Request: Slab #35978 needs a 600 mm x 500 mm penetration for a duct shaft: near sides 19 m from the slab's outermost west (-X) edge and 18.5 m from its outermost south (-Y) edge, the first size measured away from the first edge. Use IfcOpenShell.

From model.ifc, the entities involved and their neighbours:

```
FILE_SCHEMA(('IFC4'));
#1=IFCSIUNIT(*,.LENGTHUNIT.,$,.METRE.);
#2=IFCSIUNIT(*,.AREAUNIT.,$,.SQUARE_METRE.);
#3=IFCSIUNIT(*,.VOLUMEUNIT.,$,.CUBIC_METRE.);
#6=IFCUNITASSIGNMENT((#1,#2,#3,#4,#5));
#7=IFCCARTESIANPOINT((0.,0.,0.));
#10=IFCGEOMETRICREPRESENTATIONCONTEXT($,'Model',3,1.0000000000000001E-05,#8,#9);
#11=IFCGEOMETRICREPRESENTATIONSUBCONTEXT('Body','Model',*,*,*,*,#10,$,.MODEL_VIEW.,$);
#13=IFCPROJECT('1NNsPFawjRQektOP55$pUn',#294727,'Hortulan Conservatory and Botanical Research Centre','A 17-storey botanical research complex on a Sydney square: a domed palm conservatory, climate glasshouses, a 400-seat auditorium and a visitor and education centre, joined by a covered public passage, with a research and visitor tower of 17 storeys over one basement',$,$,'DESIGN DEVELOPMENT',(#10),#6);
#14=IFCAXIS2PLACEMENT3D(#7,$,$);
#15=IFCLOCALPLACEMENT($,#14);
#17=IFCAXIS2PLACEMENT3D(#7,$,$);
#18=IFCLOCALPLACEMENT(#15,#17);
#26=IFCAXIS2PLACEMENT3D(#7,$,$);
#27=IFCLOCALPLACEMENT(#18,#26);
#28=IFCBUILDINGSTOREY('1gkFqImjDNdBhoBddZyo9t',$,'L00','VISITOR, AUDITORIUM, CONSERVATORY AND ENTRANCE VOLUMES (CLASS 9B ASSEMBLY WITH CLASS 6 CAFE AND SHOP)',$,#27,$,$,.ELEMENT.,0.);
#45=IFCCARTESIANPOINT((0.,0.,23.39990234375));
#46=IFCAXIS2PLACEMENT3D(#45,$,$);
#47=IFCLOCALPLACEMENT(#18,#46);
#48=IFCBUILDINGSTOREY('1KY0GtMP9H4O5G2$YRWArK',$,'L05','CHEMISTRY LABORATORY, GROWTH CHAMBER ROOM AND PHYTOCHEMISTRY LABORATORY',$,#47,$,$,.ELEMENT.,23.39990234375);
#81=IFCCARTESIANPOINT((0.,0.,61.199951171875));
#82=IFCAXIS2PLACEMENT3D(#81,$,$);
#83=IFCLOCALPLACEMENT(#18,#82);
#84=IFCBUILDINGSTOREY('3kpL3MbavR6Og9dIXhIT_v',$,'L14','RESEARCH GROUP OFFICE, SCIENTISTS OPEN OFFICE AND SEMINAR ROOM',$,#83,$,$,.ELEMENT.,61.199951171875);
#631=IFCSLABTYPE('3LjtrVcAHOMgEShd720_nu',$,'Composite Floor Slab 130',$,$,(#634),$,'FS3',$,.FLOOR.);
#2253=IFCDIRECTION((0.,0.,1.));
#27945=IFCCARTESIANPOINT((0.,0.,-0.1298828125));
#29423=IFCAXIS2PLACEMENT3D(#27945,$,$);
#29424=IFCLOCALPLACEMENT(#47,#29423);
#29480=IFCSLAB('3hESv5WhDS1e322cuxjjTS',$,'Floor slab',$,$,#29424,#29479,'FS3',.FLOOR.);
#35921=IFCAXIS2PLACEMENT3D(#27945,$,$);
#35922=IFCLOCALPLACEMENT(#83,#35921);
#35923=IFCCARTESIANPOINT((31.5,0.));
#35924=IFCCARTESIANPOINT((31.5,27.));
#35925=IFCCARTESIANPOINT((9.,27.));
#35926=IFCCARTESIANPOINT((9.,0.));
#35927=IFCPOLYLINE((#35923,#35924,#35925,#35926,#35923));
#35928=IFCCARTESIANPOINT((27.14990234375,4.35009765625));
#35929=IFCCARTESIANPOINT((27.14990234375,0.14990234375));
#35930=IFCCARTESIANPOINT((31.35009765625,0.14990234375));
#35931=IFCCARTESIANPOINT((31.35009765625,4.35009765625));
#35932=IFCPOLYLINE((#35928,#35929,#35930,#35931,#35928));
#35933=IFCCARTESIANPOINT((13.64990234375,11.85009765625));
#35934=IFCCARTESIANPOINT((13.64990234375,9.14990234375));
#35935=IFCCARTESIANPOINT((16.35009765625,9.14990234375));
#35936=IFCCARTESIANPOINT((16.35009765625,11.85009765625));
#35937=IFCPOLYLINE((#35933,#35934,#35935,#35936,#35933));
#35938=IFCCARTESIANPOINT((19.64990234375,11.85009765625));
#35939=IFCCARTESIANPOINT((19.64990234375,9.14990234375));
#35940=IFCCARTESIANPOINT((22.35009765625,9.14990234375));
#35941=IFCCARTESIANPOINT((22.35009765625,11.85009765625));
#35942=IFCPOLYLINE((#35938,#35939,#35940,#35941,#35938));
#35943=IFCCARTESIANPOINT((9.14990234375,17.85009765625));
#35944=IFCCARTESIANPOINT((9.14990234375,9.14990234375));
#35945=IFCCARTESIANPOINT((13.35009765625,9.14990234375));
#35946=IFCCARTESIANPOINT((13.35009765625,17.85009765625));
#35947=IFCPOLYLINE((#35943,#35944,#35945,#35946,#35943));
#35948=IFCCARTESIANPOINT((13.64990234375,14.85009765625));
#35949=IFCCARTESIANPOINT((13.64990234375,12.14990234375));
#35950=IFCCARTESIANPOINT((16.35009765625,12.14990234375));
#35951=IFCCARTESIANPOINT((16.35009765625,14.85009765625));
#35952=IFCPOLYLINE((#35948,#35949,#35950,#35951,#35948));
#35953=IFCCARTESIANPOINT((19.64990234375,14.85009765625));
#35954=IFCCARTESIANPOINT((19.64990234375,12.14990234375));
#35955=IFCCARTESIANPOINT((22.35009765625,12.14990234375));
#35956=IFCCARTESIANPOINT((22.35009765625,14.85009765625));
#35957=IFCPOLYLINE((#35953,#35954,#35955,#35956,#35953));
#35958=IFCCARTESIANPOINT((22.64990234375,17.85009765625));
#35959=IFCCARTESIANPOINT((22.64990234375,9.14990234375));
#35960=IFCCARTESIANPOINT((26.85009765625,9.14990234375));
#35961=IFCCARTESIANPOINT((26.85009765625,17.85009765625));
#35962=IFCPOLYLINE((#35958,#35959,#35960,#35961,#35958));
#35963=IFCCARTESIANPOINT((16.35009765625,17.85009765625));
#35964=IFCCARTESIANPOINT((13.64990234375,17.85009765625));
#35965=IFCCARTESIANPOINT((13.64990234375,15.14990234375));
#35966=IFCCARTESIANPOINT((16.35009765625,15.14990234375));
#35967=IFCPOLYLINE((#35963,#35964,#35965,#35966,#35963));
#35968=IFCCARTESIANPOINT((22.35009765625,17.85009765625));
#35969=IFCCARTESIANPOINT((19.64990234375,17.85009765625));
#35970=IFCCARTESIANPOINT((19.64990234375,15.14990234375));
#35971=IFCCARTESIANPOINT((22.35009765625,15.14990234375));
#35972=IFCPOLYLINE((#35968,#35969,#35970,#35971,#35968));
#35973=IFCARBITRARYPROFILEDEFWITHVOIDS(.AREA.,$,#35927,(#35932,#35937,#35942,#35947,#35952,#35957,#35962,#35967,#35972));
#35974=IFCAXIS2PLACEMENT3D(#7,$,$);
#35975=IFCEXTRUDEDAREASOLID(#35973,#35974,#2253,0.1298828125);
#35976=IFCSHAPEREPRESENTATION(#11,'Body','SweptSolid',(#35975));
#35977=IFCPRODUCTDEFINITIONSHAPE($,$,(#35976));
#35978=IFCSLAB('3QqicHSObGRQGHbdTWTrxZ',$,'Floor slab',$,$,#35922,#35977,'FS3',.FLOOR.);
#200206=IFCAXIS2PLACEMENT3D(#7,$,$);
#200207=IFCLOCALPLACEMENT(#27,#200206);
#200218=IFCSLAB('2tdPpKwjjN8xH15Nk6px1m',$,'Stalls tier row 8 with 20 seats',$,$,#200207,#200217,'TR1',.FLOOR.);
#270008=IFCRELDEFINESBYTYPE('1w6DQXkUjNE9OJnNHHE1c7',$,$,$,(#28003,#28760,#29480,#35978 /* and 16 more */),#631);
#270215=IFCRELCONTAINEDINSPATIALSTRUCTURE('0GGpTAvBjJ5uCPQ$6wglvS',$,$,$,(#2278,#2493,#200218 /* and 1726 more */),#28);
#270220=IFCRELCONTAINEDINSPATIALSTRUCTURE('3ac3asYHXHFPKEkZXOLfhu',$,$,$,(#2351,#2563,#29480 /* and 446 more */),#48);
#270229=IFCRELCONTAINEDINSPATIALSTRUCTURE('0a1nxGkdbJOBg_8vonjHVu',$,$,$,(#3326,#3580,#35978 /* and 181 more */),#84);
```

```python
import numpy as np
import ifcopenshell
import ifcopenshell.api.feature
import ifcopenshell.api.geometry
import ifcopenshell.api.root
import ifcopenshell.geom
import ifcopenshell.util.placement
import ifcopenshell.util.representation
import ifcopenshell.util.shape
import ifcopenshell.util.unit

model = ifcopenshell.open("model.ifc")
unit_scale = ifcopenshell.util.unit.calculate_unit_scale(model)
settings = ifcopenshell.geom.settings()


def volume(element):
    """Net volume in cubic metres, openings subtracted."""
    shape = ifcopenshell.geom.create_shape(settings, element)
    return ifcopenshell.util.shape.get_volume(shape.geometry)


slab = model.by_id(35978)
before = volume(slab)

# Extent in the slab's own axes, in metres. The edges named are its -X and -Y sides.
slab_shape = ifcopenshell.geom.create_shape(settings, slab)
vertices = ifcopenshell.util.shape.get_vertices(slab_shape.geometry)
x_min, y_min, bottom = vertices.min(axis=0)
top = vertices[:, 2].max()

opening = ifcopenshell.api.root.create_entity(model, ifc_class="IfcOpeningElement", name="Duct shaft opening", predefined_type="OPENING")
context = ifcopenshell.util.representation.get_context(model, "Model", "Body", "MODEL_VIEW")
width, depth = 0.6, 0.5
outline = [(0.0, 0.0), (width, 0.0), (width, depth), (0.0, depth), (0.0, 0.0)]
# Overshoot both faces by 50 mm so the cut is clean.
shape = ifcopenshell.api.geometry.add_slab_representation(
    model, context=context, depth=top - bottom + 0.1, polyline=outline
)
ifcopenshell.api.geometry.assign_representation(model, product=opening, representation=shape)

matrix = ifcopenshell.util.placement.get_local_placement(slab.ObjectPlacement)
matrix[:, 3] = matrix @ np.append(np.array([x_min + 19, y_min + 18.5, bottom - 0.05]) / unit_scale, 1.0)
ifcopenshell.api.geometry.edit_object_placement(model, product=opening, matrix=matrix, is_si=False)
ifcopenshell.api.feature.add_feature(model, feature=opening, element=slab)

after = volume(slab)

print(f"slab volume {before:.3f} -> {after:.3f} m3")

model.write("model_updated.ifc")
```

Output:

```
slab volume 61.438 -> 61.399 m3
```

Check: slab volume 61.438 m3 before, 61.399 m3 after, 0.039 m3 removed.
